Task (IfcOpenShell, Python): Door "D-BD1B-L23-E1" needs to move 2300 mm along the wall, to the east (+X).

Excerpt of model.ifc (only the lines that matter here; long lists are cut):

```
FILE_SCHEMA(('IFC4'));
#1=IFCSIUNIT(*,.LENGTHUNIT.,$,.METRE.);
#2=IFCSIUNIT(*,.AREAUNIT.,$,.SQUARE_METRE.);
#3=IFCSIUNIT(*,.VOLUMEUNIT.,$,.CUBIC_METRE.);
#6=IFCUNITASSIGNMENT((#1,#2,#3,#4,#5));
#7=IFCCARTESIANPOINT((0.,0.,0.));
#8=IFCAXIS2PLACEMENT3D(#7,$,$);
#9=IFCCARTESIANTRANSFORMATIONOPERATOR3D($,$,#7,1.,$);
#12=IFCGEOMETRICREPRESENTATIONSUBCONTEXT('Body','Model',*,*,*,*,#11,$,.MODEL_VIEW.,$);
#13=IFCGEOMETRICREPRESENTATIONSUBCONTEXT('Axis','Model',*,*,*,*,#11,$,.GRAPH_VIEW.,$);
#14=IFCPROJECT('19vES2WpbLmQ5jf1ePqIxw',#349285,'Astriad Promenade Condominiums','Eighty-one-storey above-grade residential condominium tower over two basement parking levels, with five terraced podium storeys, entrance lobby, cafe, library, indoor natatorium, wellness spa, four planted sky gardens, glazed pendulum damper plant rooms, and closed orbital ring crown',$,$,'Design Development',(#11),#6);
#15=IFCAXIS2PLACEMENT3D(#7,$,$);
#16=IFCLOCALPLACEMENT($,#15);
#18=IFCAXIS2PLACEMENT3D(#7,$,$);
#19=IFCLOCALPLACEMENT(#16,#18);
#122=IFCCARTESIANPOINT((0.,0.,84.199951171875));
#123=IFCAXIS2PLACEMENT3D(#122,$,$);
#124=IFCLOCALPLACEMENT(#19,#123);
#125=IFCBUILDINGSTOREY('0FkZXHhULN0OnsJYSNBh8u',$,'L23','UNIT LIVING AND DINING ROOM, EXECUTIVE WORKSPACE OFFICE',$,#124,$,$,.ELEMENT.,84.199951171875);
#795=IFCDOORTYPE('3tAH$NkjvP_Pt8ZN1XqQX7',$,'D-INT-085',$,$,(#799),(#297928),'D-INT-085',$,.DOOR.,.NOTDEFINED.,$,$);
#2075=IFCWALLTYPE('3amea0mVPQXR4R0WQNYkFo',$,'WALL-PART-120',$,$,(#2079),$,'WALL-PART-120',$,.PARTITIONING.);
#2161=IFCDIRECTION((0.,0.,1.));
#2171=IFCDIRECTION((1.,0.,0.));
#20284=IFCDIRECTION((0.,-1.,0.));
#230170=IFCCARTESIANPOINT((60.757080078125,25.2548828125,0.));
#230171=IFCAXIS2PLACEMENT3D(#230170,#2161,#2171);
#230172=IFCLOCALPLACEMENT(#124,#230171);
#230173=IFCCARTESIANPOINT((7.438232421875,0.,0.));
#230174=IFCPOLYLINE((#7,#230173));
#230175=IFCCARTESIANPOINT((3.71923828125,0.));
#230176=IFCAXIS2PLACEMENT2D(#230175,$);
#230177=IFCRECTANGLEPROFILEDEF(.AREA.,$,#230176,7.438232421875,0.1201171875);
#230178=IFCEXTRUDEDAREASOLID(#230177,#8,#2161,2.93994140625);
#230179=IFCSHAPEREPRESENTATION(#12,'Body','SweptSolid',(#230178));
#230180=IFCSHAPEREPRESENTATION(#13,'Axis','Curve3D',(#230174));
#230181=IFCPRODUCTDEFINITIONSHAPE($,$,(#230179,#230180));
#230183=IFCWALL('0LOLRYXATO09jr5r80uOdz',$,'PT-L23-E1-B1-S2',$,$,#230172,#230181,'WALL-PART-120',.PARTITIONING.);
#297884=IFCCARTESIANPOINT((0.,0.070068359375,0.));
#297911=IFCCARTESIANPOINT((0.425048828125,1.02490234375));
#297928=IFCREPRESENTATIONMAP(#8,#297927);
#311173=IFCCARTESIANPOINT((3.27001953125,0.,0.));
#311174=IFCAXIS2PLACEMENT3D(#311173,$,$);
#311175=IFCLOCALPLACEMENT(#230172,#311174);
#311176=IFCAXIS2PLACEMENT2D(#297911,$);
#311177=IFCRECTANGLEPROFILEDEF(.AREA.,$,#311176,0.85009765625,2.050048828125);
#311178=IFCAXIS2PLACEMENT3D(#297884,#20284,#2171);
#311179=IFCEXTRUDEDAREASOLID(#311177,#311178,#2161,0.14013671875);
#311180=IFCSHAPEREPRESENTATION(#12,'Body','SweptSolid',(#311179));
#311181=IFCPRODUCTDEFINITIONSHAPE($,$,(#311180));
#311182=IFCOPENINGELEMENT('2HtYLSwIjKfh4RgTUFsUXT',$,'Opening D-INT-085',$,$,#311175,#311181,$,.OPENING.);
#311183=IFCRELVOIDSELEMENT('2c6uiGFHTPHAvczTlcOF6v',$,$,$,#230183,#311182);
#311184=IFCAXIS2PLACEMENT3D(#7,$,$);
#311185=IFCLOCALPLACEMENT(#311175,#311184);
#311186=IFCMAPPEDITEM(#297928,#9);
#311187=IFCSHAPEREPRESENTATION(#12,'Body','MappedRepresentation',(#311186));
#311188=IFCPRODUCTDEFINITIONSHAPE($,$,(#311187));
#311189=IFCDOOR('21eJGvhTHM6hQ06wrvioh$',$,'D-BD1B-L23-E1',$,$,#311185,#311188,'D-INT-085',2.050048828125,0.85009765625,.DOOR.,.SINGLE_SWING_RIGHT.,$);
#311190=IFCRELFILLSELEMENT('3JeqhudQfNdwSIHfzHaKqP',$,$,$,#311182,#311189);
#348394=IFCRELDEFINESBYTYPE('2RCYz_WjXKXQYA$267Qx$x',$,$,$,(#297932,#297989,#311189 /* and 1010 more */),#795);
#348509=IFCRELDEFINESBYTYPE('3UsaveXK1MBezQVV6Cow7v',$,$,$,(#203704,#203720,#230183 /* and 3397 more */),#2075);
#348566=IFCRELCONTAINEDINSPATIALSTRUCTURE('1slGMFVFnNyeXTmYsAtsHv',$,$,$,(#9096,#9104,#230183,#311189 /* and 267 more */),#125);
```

```python
import ifcopenshell
import ifcopenshell.api.geometry
import ifcopenshell.util.placement

model = ifcopenshell.open("model.ifc")

door = model.by_guid("21eJGvhTHM6hQ06wrvioh$")
opening = door.FillsVoids[0].RelatingOpeningElement
wall = opening.VoidsElements[0].RelatingBuildingElement

wall_matrix = ifcopenshell.util.placement.get_local_placement(wall.ObjectPlacement)
shift = wall_matrix[:3, 0] * 2.3
before = ifcopenshell.util.placement.get_local_placement(door.ObjectPlacement)[:3, 3].copy()

# The door is placed relative to its opening, so it follows when the opening moves.
matrix = ifcopenshell.util.placement.get_local_placement(opening.ObjectPlacement)
matrix[:3, 3] += shift
ifcopenshell.api.geometry.edit_object_placement(
    model, product=opening, matrix=matrix, is_si=False, should_transform_children=True
)

after = ifcopenshell.util.placement.get_local_placement(door.ObjectPlacement)[:3, 3]
print("door moved by", (after - before).round(3) + 0.0)

model.write("model_updated.ifc")
```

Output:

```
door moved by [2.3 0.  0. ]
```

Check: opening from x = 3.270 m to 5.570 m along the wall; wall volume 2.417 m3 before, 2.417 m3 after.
